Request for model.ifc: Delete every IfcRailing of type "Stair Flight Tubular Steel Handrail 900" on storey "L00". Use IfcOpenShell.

First a look at what the model holds.

```python
import ifcopenshell
import ifcopenshell.util.element

model = ifcopenshell.open("model.ifc")
print(model.schema)
storey = next(s for s in model.by_type("IfcBuildingStorey") if s.Name == "L00")
railings = [e for e in ifcopenshell.util.element.get_decomposition(storey) if e.is_a("IfcRailing")]
seen = {}
for e in railings:
    element_type = ifcopenshell.util.element.get_type(e)
    name = element_type.Name if element_type not in (None, e) else None
    seen[name] = seen.get(name, 0) + 1
for name, count in sorted(seen.items(), key=str):
    print(count, "x", name)
```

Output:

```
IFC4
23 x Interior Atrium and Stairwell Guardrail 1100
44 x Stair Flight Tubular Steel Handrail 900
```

```python
import ifcopenshell
import ifcopenshell.api.root
import ifcopenshell.util.element

model = ifcopenshell.open("model.ifc")

storey = next(s for s in model.by_type("IfcBuildingStorey") if s.Name == "L00")
railings = [e for e in ifcopenshell.util.element.get_decomposition(storey) if e.is_a("IfcRailing")]
targets = [e for e in railings if (t := ifcopenshell.util.element.get_type(e)) not in (None, e) and t.Name == "Stair Flight Tubular Steel Handrail 900"]

for e in targets:
    ifcopenshell.api.root.remove_product(model, product=e)
print(len(targets), "removed")

model.write("model_edited.ifc")
```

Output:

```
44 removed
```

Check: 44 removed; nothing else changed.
